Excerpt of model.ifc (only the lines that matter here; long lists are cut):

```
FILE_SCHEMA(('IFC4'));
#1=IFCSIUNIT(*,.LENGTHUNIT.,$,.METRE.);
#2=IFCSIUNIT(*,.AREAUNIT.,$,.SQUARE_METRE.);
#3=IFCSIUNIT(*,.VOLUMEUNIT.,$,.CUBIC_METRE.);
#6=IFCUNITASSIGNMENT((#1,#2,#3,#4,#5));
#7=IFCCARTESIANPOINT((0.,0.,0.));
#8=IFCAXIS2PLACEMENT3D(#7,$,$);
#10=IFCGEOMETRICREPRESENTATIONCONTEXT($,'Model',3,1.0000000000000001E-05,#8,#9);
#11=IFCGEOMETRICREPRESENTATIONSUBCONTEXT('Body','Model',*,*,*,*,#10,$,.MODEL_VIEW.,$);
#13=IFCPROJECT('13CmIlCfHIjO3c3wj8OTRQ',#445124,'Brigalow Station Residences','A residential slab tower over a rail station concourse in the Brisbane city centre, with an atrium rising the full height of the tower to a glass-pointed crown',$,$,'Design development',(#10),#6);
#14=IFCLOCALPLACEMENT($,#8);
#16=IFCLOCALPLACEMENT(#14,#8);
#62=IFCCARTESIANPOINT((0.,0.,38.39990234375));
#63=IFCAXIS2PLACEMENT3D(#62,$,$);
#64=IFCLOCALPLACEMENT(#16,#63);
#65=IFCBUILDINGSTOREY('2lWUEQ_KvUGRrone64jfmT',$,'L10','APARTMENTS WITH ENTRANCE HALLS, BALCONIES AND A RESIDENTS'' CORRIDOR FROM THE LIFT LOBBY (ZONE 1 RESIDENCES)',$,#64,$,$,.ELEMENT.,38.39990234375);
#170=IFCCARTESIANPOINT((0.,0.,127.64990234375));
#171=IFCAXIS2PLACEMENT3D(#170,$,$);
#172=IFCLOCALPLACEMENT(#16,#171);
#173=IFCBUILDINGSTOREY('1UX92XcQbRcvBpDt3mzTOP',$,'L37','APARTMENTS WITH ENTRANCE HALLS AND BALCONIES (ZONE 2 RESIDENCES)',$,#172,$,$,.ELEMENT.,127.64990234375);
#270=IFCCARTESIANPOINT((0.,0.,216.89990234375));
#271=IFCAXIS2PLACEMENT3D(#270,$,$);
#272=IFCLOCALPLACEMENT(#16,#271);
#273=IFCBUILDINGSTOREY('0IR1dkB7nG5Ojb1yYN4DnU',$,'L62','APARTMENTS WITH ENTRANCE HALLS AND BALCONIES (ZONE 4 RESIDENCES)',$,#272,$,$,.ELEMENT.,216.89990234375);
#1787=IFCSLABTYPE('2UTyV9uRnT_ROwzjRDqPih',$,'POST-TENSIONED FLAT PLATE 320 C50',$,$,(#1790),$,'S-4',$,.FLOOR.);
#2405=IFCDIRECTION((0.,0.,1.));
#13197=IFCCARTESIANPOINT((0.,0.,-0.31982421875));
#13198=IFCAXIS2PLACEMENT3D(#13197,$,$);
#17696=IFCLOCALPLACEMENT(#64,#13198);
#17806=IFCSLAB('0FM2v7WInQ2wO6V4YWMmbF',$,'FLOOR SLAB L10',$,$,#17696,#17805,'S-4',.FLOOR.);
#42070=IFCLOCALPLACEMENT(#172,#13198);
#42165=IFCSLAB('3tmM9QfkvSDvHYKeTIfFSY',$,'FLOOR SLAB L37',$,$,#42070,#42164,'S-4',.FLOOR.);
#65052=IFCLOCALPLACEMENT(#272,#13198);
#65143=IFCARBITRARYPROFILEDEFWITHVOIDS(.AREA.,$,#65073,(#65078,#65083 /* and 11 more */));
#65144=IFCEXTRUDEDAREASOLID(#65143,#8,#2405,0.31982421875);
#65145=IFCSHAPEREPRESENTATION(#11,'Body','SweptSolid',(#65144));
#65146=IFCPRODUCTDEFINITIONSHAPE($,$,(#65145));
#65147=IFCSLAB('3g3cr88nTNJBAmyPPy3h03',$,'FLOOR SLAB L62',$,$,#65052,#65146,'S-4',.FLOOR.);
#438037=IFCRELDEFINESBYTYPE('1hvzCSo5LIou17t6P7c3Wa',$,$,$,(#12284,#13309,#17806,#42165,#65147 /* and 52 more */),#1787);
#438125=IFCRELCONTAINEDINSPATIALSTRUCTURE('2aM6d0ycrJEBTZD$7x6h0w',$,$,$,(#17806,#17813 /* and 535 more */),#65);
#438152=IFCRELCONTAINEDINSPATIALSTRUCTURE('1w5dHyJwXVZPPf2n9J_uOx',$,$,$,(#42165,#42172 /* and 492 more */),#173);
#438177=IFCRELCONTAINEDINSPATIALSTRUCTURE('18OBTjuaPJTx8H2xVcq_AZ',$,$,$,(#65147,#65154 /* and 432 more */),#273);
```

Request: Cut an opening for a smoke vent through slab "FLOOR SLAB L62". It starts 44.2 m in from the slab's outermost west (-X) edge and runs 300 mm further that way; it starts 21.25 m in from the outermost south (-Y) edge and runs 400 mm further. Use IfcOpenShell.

```python
import numpy as np
import ifcopenshell
import ifcopenshell.api.feature
import ifcopenshell.api.geometry
import ifcopenshell.api.root
import ifcopenshell.geom
import ifcopenshell.util.placement
import ifcopenshell.util.representation
import ifcopenshell.util.shape
import ifcopenshell.util.unit

model = ifcopenshell.open("model.ifc")
unit_scale = ifcopenshell.util.unit.calculate_unit_scale(model)
settings = ifcopenshell.geom.settings()


def volume(element):
    """Net volume in cubic metres, openings subtracted."""
    shape = ifcopenshell.geom.create_shape(settings, element)
    return ifcopenshell.util.shape.get_volume(shape.geometry)


slab = model.by_guid("3g3cr88nTNJBAmyPPy3h03")
before = volume(slab)

# Extent in the slab's own axes, in metres. The edges named are its -X and -Y sides.
slab_shape = ifcopenshell.geom.create_shape(settings, slab)
vertices = ifcopenshell.util.shape.get_vertices(slab_shape.geometry)
x_min, y_min, bottom = vertices.min(axis=0)
top = vertices[:, 2].max()

opening = ifcopenshell.api.root.create_entity(model, ifc_class="IfcOpeningElement", name="Smoke vent opening", predefined_type="OPENING")
context = ifcopenshell.util.representation.get_context(model, "Model", "Body", "MODEL_VIEW")
width, depth = 0.3, 0.4
outline = [(0.0, 0.0), (width, 0.0), (width, depth), (0.0, depth), (0.0, 0.0)]
# Overshoot both faces by 50 mm so the cut is clean.
shape = ifcopenshell.api.geometry.add_slab_representation(
    model, context=context, depth=top - bottom + 0.1, polyline=outline
)
ifcopenshell.api.geometry.assign_representation(model, product=opening, representation=shape)

matrix = ifcopenshell.util.placement.get_local_placement(slab.ObjectPlacement)
matrix[:, 3] = matrix @ np.append(np.array([x_min + 44.2, y_min + 21.25, bottom - 0.05]) / unit_scale, 1.0)
ifcopenshell.api.geometry.edit_object_placement(model, product=opening, matrix=matrix, is_si=False)
ifcopenshell.api.feature.add_feature(model, feature=opening, element=slab)

after = volume(slab)

print(f"slab volume {before:.3f} -> {after:.3f} m3")

model.write("model_updated.ifc")
```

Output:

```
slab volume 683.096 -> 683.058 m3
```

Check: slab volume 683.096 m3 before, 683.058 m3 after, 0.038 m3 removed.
